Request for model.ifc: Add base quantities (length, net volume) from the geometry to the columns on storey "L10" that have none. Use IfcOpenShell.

First a look at what the model holds.

```python
import ifcopenshell
import ifcopenshell.util.element
import ifcopenshell.util.unit

model = ifcopenshell.open("model.ifc")
print(model.schema)
for unit_type in ("LENGTHUNIT", "AREAUNIT", "VOLUMEUNIT"):
    print(unit_type, ifcopenshell.util.unit.calculate_unit_scale(model, unit_type))
storey = next(s for s in model.by_type("IfcBuildingStorey") if s.Name == "L10")
columns = [e for e in ifcopenshell.util.element.get_decomposition(storey) if e.is_a("IfcColumn")]
for e in sorted(columns, key=lambda e: e.id()):
    print(e.id(), e.is_a(), e.Name, list(ifcopenshell.util.element.get_psets(e, qtos_only=True)), sep=" | ")
```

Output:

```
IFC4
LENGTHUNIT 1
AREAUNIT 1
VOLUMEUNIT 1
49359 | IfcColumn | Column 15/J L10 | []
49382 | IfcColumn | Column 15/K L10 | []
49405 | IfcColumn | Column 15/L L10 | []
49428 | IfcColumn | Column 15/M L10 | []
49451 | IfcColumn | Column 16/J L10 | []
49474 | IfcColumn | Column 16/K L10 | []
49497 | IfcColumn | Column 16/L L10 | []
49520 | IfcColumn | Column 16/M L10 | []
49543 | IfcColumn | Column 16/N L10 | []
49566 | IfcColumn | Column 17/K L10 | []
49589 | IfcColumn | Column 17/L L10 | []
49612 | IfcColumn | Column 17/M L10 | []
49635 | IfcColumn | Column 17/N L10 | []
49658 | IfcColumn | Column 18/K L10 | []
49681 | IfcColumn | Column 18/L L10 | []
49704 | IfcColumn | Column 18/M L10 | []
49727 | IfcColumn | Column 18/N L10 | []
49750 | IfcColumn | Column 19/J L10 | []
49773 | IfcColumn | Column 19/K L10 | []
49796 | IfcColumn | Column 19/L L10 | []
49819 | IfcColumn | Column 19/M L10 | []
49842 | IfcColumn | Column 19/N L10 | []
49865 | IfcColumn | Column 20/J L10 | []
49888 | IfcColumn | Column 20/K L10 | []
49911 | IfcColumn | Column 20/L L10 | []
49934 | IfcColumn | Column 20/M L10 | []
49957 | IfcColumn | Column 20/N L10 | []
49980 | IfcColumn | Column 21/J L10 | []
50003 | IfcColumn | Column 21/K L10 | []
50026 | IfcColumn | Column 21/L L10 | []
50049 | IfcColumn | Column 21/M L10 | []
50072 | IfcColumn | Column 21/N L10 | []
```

```python
import ifcopenshell
import ifcopenshell.api.pset
import ifcopenshell.geom
import ifcopenshell.util.element
import ifcopenshell.util.shape
import ifcopenshell.util.unit

model = ifcopenshell.open("model.ifc")
unit_scale = ifcopenshell.util.unit.calculate_unit_scale(model)
volume_scale = ifcopenshell.util.unit.calculate_unit_scale(model, "VOLUMEUNIT")
settings = ifcopenshell.geom.settings()

storey = next(s for s in model.by_type("IfcBuildingStorey") if s.Name == "L10")
columns = [e for e in ifcopenshell.util.element.get_decomposition(storey) if e.is_a("IfcColumn")]

for e in sorted(columns, key=lambda e: e.id()):
    if ifcopenshell.util.element.get_psets(e, qtos_only=True, should_inherit=False):
        continue
    # Geometry comes back in metres, in the element's own axes.
    shape = ifcopenshell.geom.create_shape(settings, e)
    values = {
        "Length": ifcopenshell.util.shape.get_z(shape.geometry) / unit_scale,
        "NetVolume": ifcopenshell.util.shape.get_volume(shape.geometry) / volume_scale,
    }
    qto = ifcopenshell.api.pset.add_qto(model, product=e, name="Qto_ColumnBaseQuantities")
    ifcopenshell.api.pset.edit_qto(model, qto=qto, properties=values)
    print(e.id(), {k: round(v, 3) for k, v in values.items()})

model.write("model_rev.ifc")
```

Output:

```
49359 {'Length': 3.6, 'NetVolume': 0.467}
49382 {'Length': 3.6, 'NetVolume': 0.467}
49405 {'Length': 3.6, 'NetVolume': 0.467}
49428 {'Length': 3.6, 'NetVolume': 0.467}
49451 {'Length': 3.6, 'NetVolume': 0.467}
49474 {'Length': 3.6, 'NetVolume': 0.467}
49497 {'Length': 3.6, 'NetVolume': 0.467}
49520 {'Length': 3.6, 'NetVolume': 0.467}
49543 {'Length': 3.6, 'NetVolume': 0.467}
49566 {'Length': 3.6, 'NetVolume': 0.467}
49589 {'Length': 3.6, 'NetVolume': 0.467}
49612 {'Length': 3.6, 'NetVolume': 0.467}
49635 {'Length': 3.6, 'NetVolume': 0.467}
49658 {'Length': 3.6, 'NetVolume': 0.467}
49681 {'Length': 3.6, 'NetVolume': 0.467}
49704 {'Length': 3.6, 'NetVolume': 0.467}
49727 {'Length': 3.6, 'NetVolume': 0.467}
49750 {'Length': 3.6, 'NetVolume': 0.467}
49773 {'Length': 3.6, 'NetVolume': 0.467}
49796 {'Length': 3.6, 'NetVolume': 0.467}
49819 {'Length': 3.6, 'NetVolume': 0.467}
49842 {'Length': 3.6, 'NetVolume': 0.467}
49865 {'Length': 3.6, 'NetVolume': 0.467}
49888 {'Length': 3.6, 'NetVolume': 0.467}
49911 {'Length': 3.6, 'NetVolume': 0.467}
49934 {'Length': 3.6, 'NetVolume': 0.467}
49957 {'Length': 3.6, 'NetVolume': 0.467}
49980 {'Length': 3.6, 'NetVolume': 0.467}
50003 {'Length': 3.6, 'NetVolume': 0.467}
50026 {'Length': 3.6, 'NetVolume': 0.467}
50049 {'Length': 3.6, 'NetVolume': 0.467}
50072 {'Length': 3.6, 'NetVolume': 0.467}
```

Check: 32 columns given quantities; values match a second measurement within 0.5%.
